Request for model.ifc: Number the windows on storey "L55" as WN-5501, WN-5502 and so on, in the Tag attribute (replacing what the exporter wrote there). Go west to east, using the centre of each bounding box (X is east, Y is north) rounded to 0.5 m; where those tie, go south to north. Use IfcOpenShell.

First a look at what the model holds.

```python
import ifcopenshell
import ifcopenshell.util.element
import ifcopenshell.util.placement

model = ifcopenshell.open("model.ifc")
print(model.schema)
storey = next(s for s in model.by_type("IfcBuildingStorey") if s.Name == "L55")
windows = [e for e in ifcopenshell.util.element.get_decomposition(storey) if e.is_a("IfcWindow")]
for e in sorted(windows, key=lambda e: e.id()):
    origin = ifcopenshell.util.placement.get_local_placement(e.ObjectPlacement)[:3, 3]
    print(e.id(), e.Tag, e.Name, origin.round(2) + 0.0, sep=" | ")
```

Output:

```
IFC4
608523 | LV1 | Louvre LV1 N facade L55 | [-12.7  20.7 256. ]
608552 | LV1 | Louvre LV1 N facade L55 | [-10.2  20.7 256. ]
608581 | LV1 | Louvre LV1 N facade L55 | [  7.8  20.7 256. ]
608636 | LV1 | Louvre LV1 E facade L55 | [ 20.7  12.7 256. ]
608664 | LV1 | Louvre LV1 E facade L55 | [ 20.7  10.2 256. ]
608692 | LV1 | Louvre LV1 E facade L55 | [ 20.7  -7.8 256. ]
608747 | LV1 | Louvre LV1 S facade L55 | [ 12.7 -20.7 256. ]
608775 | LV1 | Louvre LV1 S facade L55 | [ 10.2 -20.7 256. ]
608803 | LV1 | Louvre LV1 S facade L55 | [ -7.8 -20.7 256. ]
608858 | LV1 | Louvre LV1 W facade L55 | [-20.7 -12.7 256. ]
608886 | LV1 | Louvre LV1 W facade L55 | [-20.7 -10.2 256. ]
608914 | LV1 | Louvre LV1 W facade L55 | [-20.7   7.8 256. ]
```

```python
import ifcopenshell
import ifcopenshell.geom
import ifcopenshell.util.element
import ifcopenshell.util.shape

model = ifcopenshell.open("model.ifc")
settings = ifcopenshell.geom.settings()
settings.set("use-world-coords", True)


def centre(element):
    shape = ifcopenshell.geom.create_shape(settings, element)
    return ifcopenshell.util.shape.get_bbox_centroid(shape.geometry)


storey = next(s for s in model.by_type("IfcBuildingStorey") if s.Name == "L55")
windows = [e for e in ifcopenshell.util.element.get_decomposition(storey) if e.is_a("IfcWindow")]

# Insertion points can sit at a corner or the storey origin, so sort by the geometry (in metres).
centres = {e: centre(e) for e in windows}
windows.sort(key=lambda e: (round(centres[e][0] / 0.5), centres[e][1]))

for i, e in enumerate(windows, start=1):
    number = f"WN-55{i:02d}"
    e.Tag = number
    print(e.id(), number)

model.write("model_edited.ifc")
```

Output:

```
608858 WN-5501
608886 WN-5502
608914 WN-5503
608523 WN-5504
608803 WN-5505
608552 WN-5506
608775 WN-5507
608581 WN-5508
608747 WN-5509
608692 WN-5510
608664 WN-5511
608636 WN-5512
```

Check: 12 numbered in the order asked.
